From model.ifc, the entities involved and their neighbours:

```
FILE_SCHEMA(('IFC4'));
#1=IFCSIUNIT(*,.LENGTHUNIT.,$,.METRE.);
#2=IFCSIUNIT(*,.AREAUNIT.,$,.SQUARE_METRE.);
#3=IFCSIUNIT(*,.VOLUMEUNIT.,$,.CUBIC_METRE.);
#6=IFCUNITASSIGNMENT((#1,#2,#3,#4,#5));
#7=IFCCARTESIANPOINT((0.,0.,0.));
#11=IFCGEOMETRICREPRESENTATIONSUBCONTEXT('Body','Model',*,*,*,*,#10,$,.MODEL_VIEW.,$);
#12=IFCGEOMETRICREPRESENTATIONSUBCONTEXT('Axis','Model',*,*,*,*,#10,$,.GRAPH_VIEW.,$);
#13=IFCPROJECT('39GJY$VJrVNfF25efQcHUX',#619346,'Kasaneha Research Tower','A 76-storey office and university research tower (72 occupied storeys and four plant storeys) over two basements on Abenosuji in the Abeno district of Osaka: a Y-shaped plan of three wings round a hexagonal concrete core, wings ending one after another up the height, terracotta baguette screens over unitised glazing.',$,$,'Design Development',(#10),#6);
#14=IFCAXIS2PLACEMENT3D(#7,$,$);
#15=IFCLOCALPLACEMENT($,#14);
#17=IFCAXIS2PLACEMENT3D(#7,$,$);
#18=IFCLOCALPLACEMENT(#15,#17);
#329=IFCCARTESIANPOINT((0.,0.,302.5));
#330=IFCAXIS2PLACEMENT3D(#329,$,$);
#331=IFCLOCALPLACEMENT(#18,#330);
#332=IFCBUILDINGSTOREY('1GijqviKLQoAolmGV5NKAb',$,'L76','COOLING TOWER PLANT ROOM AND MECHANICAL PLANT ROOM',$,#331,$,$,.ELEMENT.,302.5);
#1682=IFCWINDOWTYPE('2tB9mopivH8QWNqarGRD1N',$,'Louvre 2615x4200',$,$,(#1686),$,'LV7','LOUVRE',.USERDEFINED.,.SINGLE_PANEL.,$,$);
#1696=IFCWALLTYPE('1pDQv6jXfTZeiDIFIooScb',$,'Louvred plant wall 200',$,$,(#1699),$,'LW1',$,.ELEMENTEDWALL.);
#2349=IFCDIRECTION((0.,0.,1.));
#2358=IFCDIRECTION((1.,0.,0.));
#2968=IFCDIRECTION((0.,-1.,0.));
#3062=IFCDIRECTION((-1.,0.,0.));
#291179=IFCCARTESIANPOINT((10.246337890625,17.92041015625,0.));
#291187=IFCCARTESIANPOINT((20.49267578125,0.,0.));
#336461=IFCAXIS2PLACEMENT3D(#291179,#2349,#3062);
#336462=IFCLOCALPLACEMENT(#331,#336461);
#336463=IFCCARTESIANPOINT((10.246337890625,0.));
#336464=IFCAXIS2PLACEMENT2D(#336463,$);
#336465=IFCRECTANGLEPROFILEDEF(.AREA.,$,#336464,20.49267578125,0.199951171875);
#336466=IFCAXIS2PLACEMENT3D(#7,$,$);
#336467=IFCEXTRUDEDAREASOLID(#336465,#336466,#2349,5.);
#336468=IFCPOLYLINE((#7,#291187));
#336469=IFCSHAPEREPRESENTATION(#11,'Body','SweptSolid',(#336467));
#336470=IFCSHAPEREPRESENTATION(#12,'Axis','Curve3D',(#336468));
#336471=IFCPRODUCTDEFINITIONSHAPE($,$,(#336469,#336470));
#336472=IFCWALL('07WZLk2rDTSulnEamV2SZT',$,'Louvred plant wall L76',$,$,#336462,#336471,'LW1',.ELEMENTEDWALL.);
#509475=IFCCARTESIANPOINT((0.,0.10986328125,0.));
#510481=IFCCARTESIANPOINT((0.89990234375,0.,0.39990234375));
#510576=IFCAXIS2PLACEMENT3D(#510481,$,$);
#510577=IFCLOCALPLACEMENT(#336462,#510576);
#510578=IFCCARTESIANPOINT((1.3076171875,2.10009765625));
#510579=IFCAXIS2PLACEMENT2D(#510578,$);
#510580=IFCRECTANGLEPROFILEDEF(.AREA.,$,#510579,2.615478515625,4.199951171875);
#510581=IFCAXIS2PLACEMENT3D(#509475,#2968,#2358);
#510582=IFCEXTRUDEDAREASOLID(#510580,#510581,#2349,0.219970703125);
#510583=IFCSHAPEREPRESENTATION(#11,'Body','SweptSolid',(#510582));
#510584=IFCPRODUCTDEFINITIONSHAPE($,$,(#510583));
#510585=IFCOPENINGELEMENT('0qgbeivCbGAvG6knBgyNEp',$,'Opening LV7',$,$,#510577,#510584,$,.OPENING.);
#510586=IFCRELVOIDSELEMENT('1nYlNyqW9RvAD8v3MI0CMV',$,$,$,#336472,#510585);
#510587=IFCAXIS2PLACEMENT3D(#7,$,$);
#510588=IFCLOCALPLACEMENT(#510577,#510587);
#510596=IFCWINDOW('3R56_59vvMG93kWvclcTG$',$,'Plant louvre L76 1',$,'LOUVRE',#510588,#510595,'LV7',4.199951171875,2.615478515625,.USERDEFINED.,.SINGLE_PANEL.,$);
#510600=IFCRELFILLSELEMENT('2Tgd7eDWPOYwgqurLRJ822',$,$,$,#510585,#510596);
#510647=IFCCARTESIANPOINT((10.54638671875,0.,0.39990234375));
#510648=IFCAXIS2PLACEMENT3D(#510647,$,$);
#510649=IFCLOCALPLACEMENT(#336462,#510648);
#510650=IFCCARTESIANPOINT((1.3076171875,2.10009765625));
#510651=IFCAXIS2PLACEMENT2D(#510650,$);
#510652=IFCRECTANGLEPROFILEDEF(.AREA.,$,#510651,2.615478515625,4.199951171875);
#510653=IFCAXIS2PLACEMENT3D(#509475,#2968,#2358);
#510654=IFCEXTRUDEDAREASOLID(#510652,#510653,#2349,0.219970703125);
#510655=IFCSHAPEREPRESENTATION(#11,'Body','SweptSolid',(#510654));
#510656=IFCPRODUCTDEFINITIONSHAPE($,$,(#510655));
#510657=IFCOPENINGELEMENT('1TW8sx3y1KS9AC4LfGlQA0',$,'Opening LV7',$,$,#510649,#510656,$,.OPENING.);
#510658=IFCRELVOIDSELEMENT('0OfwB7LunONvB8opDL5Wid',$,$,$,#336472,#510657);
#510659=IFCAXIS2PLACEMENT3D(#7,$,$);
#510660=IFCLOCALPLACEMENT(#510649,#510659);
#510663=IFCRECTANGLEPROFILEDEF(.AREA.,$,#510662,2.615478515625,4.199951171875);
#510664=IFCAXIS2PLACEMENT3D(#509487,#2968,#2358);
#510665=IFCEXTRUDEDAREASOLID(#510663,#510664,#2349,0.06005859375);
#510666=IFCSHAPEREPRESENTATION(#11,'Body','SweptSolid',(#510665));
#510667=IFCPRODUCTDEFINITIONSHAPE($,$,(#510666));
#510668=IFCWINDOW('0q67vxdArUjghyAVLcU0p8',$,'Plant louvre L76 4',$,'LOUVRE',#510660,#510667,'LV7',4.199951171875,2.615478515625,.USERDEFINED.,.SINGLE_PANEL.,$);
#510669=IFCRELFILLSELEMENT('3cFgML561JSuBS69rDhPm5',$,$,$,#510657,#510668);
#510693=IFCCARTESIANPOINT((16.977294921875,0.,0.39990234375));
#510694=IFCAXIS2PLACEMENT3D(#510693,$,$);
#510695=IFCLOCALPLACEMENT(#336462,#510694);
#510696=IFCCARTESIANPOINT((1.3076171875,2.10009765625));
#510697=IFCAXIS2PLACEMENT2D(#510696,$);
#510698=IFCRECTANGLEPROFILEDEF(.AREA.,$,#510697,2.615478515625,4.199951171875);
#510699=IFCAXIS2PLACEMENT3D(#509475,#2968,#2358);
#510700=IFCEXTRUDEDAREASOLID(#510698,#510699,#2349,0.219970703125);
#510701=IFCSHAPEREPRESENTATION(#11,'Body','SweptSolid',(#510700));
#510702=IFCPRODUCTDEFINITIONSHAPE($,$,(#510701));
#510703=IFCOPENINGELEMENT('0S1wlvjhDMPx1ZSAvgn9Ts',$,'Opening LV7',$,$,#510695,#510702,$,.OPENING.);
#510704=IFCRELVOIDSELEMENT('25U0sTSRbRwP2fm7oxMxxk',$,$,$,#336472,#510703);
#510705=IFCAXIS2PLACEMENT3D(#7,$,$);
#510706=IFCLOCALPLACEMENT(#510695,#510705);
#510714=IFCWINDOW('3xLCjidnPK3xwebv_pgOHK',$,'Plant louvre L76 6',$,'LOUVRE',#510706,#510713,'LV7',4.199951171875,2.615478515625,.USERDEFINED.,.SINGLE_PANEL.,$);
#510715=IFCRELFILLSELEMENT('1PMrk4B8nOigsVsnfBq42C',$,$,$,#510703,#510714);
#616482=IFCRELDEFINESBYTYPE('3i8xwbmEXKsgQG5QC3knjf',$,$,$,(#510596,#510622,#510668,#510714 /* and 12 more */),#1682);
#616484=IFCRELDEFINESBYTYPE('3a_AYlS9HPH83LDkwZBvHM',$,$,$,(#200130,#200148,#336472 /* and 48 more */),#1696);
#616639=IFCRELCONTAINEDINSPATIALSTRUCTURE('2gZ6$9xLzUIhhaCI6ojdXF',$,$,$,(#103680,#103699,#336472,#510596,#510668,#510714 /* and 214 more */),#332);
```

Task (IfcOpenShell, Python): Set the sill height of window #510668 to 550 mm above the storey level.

```python
import numpy as np
import ifcopenshell
import ifcopenshell.api.geometry
import ifcopenshell.geom
import ifcopenshell.util.element
import ifcopenshell.util.placement
import ifcopenshell.util.shape
import ifcopenshell.util.unit

model = ifcopenshell.open("model.ifc")
unit_scale = ifcopenshell.util.unit.calculate_unit_scale(model)

window = model.by_guid("0q67vxdArUjghyAVLcU0p8")
opening = window.FillsVoids[0].RelatingOpeningElement
storey = ifcopenshell.util.element.get_container(window, ifc_class="IfcBuildingStorey")
level = ifcopenshell.util.placement.get_local_placement(storey.ObjectPlacement)[2, 3]

# The opening's origin need not be at the sill, so measure its lowest point.
shape = ifcopenshell.geom.create_shape(ifcopenshell.geom.settings(), opening)
bottom = ifcopenshell.util.shape.get_shape_bottom_elevation(shape, shape.geometry) / unit_scale
dz = level + 0.55 - bottom

shift = np.array([0.0, 0.0, dz])
# The window is placed relative to its opening, so it follows when the opening moves.
matrix = ifcopenshell.util.placement.get_local_placement(opening.ObjectPlacement)
matrix[:3, 3] += shift
ifcopenshell.api.geometry.edit_object_placement(
    model, product=opening, matrix=matrix, is_si=False, should_transform_children=True
)

print(f"moved by {dz * unit_scale:+.3f} m")

model.write("model_v2.ifc")
```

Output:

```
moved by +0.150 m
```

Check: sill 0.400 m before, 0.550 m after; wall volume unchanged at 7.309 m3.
